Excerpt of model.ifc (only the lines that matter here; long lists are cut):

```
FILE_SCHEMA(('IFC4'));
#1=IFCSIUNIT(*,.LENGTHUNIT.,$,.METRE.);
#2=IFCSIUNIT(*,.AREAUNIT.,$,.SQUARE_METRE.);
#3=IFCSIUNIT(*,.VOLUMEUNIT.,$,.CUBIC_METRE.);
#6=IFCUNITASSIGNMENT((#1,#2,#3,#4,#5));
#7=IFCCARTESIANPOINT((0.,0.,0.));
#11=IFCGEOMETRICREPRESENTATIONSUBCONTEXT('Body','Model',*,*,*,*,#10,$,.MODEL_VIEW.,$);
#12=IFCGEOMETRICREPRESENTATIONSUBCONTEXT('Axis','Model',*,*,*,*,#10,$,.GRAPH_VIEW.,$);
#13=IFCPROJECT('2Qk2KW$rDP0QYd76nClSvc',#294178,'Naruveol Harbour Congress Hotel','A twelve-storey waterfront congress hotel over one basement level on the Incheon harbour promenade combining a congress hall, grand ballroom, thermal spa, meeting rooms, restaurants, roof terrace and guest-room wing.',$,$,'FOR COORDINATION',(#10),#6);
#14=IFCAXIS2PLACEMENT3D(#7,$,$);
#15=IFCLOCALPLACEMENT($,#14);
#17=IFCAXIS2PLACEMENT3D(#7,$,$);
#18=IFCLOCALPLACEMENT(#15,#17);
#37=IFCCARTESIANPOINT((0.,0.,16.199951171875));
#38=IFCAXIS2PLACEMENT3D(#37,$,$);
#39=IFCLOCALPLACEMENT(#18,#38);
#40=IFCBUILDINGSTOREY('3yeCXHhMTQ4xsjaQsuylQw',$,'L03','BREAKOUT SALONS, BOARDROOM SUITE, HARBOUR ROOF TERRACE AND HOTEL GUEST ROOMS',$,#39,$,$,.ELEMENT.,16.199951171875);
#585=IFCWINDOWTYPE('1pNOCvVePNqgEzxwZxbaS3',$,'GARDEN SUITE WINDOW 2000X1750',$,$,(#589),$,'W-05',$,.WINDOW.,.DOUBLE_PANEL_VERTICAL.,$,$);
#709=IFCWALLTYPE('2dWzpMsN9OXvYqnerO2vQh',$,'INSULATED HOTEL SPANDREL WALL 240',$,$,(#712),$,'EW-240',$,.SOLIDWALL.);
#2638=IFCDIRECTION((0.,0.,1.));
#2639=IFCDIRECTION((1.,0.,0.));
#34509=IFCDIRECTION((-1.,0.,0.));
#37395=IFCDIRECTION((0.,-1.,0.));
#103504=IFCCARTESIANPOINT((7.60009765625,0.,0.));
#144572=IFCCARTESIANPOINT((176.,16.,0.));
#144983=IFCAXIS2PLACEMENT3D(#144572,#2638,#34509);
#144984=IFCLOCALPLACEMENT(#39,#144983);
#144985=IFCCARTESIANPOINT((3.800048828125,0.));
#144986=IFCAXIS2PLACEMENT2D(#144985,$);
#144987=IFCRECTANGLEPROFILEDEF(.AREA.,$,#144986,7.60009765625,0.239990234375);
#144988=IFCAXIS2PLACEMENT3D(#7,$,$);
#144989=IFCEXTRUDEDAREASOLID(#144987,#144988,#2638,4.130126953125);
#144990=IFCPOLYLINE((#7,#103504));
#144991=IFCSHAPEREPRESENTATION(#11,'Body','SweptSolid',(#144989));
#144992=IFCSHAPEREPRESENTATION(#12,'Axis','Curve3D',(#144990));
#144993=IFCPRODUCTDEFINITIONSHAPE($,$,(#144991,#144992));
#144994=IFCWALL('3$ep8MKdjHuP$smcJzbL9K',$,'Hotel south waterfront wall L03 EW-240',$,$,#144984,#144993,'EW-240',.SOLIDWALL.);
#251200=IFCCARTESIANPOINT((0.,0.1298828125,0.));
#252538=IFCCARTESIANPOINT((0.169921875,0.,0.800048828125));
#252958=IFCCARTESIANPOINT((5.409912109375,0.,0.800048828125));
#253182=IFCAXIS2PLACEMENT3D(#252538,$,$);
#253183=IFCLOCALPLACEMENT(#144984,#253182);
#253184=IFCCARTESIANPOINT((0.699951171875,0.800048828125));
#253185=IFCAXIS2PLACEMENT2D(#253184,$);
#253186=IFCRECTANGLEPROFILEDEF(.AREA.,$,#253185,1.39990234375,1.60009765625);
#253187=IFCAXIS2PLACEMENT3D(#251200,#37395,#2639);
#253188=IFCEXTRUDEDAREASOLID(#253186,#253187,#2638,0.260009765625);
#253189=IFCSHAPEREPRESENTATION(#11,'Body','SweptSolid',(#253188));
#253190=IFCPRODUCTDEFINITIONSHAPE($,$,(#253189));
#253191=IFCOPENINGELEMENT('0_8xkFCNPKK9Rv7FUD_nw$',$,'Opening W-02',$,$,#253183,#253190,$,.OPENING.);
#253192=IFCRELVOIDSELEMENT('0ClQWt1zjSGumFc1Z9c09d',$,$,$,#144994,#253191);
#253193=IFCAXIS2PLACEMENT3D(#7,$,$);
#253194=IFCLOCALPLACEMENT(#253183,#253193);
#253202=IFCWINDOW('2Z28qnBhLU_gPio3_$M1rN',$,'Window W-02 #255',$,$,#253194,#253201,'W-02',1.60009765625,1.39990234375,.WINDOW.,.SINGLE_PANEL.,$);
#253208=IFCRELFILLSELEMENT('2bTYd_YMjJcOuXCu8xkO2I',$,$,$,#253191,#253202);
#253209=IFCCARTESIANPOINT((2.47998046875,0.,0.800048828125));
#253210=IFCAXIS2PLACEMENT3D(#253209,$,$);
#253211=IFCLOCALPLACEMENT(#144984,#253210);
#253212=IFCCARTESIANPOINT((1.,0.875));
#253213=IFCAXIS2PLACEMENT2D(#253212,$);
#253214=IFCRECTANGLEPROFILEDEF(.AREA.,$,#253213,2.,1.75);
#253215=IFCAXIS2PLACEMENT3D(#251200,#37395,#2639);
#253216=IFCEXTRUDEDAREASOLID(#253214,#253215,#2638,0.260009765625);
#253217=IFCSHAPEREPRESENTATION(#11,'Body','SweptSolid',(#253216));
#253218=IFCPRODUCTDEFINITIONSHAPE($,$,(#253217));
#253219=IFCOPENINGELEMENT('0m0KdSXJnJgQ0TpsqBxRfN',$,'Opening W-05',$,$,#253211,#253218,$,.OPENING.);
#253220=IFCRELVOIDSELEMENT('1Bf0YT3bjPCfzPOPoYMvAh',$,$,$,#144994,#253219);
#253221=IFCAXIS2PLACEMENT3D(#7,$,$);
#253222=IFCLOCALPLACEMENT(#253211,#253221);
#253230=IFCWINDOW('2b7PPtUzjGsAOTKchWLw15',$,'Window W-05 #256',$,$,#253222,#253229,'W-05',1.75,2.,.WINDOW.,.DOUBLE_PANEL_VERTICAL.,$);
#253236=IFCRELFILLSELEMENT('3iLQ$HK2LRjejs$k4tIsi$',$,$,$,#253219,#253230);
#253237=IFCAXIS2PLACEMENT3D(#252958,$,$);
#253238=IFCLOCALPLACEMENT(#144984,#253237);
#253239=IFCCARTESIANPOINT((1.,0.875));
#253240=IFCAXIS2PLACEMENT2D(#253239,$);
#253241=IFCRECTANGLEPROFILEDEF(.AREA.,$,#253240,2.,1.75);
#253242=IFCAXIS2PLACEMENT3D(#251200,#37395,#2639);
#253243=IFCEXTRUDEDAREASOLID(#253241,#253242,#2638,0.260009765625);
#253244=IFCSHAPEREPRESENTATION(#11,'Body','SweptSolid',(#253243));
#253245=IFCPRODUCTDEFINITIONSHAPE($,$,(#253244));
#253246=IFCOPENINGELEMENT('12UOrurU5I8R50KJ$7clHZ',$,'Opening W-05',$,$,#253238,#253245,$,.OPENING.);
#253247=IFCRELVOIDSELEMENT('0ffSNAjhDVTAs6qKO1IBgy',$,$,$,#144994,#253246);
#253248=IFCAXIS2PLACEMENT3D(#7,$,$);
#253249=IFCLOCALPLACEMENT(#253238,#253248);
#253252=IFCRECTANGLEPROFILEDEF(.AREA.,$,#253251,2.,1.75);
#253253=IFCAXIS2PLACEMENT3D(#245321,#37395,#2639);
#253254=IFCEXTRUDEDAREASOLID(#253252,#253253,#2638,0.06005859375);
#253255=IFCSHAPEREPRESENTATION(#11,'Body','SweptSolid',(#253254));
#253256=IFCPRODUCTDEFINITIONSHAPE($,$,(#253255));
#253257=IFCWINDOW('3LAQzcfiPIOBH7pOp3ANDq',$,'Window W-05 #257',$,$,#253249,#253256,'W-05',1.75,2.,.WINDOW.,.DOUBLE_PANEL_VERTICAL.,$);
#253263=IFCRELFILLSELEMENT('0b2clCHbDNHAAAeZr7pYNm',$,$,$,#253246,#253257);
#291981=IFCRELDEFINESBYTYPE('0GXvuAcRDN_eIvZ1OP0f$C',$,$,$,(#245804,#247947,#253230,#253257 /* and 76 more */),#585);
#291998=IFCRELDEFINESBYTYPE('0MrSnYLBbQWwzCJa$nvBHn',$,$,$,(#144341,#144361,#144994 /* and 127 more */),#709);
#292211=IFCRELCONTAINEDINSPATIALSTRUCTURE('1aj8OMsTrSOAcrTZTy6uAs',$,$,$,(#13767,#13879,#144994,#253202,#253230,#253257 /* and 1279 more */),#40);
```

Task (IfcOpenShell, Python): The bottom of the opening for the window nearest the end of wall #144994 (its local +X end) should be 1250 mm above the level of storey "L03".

```python
import numpy as np
import ifcopenshell
import ifcopenshell.api.geometry
import ifcopenshell.geom
import ifcopenshell.util.element
import ifcopenshell.util.placement
import ifcopenshell.util.shape
import ifcopenshell.util.unit

model = ifcopenshell.open("model.ifc")
unit_scale = ifcopenshell.util.unit.calculate_unit_scale(model)

window = model.by_guid("3LAQzcfiPIOBH7pOp3ANDq")
opening = window.FillsVoids[0].RelatingOpeningElement
storey = ifcopenshell.util.element.get_container(window, ifc_class="IfcBuildingStorey")
level = ifcopenshell.util.placement.get_local_placement(storey.ObjectPlacement)[2, 3]

# The opening's origin need not be at the sill, so measure its lowest point.
shape = ifcopenshell.geom.create_shape(ifcopenshell.geom.settings(), opening)
bottom = ifcopenshell.util.shape.get_shape_bottom_elevation(shape, shape.geometry) / unit_scale
dz = level + 1.25 / unit_scale - bottom

shift = np.array([0.0, 0.0, dz])
# The window is placed relative to its opening, so it follows when the opening moves.
matrix = ifcopenshell.util.placement.get_local_placement(opening.ObjectPlacement)
matrix[:3, 3] += shift
ifcopenshell.api.geometry.edit_object_placement(
    model, product=opening, matrix=matrix, is_si=False, should_transform_children=True
)

print(f"moved by {dz * unit_scale:+.3f} m")

model.write("model_updated.ifc")
```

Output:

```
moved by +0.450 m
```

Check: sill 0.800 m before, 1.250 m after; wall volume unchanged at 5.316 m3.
